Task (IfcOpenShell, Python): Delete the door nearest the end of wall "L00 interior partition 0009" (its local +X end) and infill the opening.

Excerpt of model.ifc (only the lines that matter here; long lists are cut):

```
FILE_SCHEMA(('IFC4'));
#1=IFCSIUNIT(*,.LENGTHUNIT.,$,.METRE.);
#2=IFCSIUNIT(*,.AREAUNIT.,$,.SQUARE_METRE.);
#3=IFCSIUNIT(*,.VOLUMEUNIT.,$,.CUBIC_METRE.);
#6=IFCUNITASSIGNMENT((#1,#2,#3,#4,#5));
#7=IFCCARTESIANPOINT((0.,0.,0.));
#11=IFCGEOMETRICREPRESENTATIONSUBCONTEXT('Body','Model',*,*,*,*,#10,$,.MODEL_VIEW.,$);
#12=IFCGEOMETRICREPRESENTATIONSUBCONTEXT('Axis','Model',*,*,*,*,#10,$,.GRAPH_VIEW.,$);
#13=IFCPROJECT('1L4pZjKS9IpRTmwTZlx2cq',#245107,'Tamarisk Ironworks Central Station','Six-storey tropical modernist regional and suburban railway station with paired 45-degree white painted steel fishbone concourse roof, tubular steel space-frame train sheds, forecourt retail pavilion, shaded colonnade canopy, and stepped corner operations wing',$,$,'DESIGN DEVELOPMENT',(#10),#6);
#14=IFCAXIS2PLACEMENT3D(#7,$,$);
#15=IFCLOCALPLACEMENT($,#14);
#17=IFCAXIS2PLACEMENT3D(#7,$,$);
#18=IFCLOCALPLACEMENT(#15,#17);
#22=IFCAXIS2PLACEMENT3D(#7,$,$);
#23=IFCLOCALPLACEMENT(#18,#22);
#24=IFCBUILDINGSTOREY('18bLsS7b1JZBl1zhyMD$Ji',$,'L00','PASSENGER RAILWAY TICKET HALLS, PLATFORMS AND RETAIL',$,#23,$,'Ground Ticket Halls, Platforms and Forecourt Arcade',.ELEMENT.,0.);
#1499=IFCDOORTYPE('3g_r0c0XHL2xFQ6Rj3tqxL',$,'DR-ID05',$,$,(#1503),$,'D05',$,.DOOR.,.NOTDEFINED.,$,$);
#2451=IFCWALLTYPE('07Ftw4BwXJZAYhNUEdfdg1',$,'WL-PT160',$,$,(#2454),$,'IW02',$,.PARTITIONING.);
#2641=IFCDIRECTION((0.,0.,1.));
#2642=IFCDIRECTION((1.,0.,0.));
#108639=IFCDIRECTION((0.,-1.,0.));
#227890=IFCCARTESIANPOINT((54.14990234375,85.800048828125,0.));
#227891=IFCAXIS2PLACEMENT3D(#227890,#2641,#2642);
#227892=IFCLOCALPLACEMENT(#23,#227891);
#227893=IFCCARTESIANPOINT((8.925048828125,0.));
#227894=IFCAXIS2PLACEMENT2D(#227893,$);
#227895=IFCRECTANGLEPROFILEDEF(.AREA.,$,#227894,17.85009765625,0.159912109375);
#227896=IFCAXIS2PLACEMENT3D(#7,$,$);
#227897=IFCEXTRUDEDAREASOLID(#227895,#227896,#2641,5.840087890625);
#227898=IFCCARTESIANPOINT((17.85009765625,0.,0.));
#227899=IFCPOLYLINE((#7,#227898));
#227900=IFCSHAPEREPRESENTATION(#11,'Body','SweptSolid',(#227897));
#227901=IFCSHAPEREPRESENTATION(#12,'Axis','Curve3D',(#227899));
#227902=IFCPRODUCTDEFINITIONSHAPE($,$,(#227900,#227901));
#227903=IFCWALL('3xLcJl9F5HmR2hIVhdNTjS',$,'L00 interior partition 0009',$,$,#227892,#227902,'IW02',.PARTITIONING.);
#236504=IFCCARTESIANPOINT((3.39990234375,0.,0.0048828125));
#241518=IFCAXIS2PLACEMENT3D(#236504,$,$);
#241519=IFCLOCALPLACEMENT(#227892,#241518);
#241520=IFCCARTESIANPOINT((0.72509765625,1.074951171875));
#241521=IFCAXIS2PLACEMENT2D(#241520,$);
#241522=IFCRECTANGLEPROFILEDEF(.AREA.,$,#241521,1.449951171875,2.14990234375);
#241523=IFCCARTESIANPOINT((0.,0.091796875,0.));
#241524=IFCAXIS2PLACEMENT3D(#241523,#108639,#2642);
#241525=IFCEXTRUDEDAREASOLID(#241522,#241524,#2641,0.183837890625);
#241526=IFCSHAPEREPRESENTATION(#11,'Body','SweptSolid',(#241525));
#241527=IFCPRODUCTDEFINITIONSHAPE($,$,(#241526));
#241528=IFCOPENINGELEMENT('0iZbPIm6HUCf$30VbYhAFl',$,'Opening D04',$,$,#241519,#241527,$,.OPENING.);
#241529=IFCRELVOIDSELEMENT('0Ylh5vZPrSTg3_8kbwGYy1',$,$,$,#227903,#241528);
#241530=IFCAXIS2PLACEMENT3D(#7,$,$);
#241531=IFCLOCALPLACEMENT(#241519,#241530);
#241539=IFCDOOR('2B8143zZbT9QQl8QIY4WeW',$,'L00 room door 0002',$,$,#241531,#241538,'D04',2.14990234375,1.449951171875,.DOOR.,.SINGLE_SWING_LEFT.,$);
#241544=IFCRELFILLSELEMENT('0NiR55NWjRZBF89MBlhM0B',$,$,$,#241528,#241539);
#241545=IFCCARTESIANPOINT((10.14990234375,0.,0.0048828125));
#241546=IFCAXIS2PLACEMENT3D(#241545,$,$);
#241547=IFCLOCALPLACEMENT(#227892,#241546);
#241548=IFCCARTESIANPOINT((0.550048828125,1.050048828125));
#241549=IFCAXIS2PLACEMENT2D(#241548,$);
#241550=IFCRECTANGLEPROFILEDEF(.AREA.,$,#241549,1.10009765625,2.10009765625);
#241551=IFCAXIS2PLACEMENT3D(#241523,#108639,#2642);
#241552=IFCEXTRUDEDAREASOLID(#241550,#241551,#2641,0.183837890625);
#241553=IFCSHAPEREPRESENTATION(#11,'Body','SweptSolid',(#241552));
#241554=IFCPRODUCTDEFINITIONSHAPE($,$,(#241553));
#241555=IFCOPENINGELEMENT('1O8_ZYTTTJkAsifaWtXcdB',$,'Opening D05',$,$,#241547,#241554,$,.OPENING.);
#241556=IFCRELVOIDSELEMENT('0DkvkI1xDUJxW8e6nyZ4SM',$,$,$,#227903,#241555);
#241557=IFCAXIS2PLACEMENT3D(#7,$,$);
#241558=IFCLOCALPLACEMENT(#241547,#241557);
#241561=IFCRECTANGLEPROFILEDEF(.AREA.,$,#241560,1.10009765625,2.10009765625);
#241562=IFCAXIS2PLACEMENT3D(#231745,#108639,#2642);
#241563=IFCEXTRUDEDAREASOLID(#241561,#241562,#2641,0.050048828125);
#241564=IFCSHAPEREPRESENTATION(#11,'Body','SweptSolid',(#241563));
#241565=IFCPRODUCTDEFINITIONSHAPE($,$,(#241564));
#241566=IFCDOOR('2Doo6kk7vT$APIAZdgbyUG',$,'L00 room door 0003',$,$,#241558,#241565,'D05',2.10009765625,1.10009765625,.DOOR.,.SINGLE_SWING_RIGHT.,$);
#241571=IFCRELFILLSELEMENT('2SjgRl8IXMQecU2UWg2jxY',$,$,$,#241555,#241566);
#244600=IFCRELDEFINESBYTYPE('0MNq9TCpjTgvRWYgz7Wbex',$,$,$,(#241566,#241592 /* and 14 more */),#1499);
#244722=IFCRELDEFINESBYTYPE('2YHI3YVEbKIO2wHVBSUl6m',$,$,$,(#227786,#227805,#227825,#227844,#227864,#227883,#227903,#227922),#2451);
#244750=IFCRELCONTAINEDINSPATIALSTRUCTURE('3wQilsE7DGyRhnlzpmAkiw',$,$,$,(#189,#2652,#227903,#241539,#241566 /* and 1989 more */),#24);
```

```python
import ifcopenshell
import ifcopenshell.api.feature
import ifcopenshell.api.root
import ifcopenshell.geom
import ifcopenshell.util.shape

model = ifcopenshell.open("model.ifc")
settings = ifcopenshell.geom.settings()


def volume(element):
    """Net volume in cubic metres, openings subtracted."""
    shape = ifcopenshell.geom.create_shape(settings, element)
    return ifcopenshell.util.shape.get_volume(shape.geometry)


door = model.by_guid("2Doo6kk7vT$APIAZdgbyUG")
opening = door.FillsVoids[0].RelatingOpeningElement
wall = opening.VoidsElements[0].RelatingBuildingElement
before = volume(wall)

ifcopenshell.api.root.remove_product(model, product=door)
ifcopenshell.api.feature.remove_feature(model, feature=opening)

after = volume(wall)

print(f"wall volume {before:.3f} -> {after:.3f} m3")

model.write("model_v2.ifc")
```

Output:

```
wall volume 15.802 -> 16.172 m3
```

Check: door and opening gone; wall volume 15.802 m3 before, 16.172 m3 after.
